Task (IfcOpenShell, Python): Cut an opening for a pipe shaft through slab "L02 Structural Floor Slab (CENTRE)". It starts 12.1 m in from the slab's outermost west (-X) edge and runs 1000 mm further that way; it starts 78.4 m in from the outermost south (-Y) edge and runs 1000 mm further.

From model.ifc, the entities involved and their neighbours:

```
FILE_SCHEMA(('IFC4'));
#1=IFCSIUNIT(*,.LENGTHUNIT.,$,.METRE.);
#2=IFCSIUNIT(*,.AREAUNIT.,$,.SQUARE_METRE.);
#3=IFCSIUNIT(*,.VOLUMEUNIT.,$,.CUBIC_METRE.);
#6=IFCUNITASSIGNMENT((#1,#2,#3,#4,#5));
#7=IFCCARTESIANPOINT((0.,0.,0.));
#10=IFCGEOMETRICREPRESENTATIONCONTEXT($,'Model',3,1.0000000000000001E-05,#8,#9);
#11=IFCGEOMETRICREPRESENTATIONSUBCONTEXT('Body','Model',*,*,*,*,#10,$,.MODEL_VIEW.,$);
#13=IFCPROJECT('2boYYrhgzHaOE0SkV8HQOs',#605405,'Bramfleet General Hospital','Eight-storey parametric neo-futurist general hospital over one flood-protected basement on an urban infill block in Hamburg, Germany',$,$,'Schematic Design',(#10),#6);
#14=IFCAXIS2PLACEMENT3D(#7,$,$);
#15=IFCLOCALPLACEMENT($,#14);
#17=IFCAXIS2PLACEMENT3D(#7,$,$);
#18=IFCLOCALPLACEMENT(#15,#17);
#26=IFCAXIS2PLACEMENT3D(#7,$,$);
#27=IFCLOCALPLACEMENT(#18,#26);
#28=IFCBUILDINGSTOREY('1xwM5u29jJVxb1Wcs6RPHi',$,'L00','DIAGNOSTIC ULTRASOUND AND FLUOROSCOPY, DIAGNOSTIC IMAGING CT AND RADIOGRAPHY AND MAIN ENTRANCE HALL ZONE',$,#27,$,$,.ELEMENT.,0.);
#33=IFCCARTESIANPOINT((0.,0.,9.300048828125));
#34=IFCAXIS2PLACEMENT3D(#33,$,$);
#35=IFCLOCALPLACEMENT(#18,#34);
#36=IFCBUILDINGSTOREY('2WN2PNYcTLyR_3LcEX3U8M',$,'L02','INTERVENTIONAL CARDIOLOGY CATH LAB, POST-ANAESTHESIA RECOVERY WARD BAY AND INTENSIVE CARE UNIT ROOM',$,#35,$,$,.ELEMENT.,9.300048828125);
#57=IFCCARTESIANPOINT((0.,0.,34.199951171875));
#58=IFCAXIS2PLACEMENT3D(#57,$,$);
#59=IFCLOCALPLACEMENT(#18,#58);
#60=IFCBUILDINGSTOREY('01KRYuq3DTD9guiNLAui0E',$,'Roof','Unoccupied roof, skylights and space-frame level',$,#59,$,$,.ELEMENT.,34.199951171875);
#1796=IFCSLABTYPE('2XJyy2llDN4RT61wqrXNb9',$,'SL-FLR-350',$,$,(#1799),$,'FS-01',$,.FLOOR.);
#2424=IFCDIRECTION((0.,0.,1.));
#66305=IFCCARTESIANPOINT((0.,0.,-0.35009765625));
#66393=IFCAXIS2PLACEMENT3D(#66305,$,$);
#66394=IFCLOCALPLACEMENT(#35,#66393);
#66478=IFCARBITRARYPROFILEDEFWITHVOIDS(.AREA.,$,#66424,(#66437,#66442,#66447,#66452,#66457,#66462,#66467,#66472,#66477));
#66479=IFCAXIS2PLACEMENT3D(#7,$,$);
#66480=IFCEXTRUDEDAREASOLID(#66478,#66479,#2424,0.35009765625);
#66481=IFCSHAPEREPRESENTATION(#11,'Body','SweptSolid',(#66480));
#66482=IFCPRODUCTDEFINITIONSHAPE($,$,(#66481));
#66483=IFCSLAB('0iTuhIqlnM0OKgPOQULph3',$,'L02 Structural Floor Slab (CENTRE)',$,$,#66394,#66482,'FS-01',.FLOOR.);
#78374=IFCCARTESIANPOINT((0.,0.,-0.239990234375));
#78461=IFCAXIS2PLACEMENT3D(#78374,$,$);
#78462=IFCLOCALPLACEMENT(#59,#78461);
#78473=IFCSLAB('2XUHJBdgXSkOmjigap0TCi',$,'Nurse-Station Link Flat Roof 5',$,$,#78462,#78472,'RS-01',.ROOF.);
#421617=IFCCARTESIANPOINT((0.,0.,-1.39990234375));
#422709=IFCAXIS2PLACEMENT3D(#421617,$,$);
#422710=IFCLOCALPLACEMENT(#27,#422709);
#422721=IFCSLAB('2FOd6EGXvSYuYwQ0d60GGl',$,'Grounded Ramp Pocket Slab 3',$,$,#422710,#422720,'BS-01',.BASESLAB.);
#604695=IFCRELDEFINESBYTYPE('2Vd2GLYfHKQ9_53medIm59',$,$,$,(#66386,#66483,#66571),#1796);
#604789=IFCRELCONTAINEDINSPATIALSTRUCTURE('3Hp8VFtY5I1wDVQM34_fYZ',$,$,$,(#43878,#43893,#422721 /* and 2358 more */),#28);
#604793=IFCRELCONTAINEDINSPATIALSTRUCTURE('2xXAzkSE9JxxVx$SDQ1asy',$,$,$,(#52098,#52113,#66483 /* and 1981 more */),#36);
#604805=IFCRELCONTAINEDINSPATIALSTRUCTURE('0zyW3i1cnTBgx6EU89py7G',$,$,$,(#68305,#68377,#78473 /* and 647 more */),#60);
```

```python
import numpy as np
import ifcopenshell
import ifcopenshell.api.feature
import ifcopenshell.api.geometry
import ifcopenshell.api.root
import ifcopenshell.geom
import ifcopenshell.util.placement
import ifcopenshell.util.representation
import ifcopenshell.util.shape
import ifcopenshell.util.unit

model = ifcopenshell.open("model.ifc")
unit_scale = ifcopenshell.util.unit.calculate_unit_scale(model)
settings = ifcopenshell.geom.settings()


def volume(element):
    """Net volume in cubic metres, openings subtracted."""
    shape = ifcopenshell.geom.create_shape(settings, element)
    return ifcopenshell.util.shape.get_volume(shape.geometry)


slab = model.by_guid("0iTuhIqlnM0OKgPOQULph3")
before = volume(slab)

# Extent in the slab's own axes, in metres. The edges named are its -X and -Y sides.
slab_shape = ifcopenshell.geom.create_shape(settings, slab)
vertices = ifcopenshell.util.shape.get_vertices(slab_shape.geometry)
x_min, y_min, bottom = vertices.min(axis=0)
top = vertices[:, 2].max()

opening = ifcopenshell.api.root.create_entity(model, ifc_class="IfcOpeningElement", name="Pipe shaft opening", predefined_type="OPENING")
context = ifcopenshell.util.representation.get_context(model, "Model", "Body", "MODEL_VIEW")
width, depth = 1, 1
outline = [(0.0, 0.0), (width, 0.0), (width, depth), (0.0, depth), (0.0, 0.0)]
# Overshoot both faces by 50 mm so the cut is clean.
shape = ifcopenshell.api.geometry.add_slab_representation(
    model, context=context, depth=top - bottom + 0.1, polyline=outline
)
ifcopenshell.api.geometry.assign_representation(model, product=opening, representation=shape)

matrix = ifcopenshell.util.placement.get_local_placement(slab.ObjectPlacement)
matrix[:, 3] = matrix @ np.append(np.array([x_min + 12.1, y_min + 78.4, bottom - 0.05]) / unit_scale, 1.0)
ifcopenshell.api.geometry.edit_object_placement(model, product=opening, matrix=matrix, is_si=False)
ifcopenshell.api.feature.add_feature(model, feature=opening, element=slab)

after = volume(slab)

print(f"slab volume {before:.3f} -> {after:.3f} m3")

model.write("model_v2.ifc")
```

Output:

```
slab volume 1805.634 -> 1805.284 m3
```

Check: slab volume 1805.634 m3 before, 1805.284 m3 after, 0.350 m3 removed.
